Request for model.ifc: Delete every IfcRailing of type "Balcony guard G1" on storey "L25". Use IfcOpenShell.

First a look at what the model holds.

```python
import ifcopenshell
import ifcopenshell.util.element

model = ifcopenshell.open("model.ifc")
print(model.schema)
storey = next(s for s in model.by_type("IfcBuildingStorey") if s.Name == "L25")
railings = [e for e in ifcopenshell.util.element.get_decomposition(storey) if e.is_a("IfcRailing")]
seen = {}
for e in railings:
    element_type = ifcopenshell.util.element.get_type(e)
    name = element_type.Name if element_type not in (None, e) else None
    seen[name] = seen.get(name, 0) + 1
for name, count in sorted(seen.items(), key=str):
    print(count, "x", name)
```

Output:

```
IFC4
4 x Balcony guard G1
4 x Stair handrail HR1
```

```python
import ifcopenshell
import ifcopenshell.api.root
import ifcopenshell.util.element

model = ifcopenshell.open("model.ifc")

storey = next(s for s in model.by_type("IfcBuildingStorey") if s.Name == "L25")
railings = [e for e in ifcopenshell.util.element.get_decomposition(storey) if e.is_a("IfcRailing")]
targets = [e for e in railings if (t := ifcopenshell.util.element.get_type(e)) not in (None, e) and t.Name == "Balcony guard G1"]

for e in targets:
    ifcopenshell.api.root.remove_product(model, product=e)
print(len(targets), "removed")

model.write("model_v2.ifc")
```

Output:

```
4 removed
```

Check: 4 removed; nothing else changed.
